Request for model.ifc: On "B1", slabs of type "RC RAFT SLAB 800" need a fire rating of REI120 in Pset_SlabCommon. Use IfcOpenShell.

First a look at what the model holds.

```python
import ifcopenshell
import ifcopenshell.util.element

model = ifcopenshell.open("model.ifc")
print(model.schema)
storey = next(s for s in model.by_type("IfcBuildingStorey") if s.Name == "B1")
slabs = [e for e in ifcopenshell.util.element.get_decomposition(storey) if e.is_a("IfcSlab")]
seen = {}
for e in slabs:
    element_type = ifcopenshell.util.element.get_type(e)
    key = (element_type.Name if element_type != e and element_type else None, ifcopenshell.util.element.get_pset(e, "Pset_SlabCommon", "FireRating"))
    seen[key] = seen.get(key, 0) + 1
for (name, value), count in sorted(seen.items(), key=str):
    print(count, "x", name, "|", value)
```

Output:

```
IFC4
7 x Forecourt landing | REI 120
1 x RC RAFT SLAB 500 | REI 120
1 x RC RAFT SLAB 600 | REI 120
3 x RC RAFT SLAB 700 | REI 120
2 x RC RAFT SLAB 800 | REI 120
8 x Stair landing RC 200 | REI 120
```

```python
import ifcopenshell
import ifcopenshell.api.pset
import ifcopenshell.util.element

model = ifcopenshell.open("model.ifc")

storey = next(s for s in model.by_type("IfcBuildingStorey") if s.Name == "B1")
slabs = [e for e in ifcopenshell.util.element.get_decomposition(storey) if e.is_a("IfcSlab")]

count = 0
for e in slabs:
    element_type = ifcopenshell.util.element.get_type(e)
    if element_type in (None, e) or element_type.Name != "RC RAFT SLAB 800":
        continue
    # add_pset returns the element's existing set when there is one.
    pset = ifcopenshell.api.pset.add_pset(model, product=e, name="Pset_SlabCommon")
    ifcopenshell.api.pset.edit_pset(model, pset=pset, properties={"FireRating": "REI120"})
    count += 1

print(count, "slabs updated")

model.write("model_updated.ifc")
```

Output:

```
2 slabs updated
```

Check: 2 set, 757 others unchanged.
